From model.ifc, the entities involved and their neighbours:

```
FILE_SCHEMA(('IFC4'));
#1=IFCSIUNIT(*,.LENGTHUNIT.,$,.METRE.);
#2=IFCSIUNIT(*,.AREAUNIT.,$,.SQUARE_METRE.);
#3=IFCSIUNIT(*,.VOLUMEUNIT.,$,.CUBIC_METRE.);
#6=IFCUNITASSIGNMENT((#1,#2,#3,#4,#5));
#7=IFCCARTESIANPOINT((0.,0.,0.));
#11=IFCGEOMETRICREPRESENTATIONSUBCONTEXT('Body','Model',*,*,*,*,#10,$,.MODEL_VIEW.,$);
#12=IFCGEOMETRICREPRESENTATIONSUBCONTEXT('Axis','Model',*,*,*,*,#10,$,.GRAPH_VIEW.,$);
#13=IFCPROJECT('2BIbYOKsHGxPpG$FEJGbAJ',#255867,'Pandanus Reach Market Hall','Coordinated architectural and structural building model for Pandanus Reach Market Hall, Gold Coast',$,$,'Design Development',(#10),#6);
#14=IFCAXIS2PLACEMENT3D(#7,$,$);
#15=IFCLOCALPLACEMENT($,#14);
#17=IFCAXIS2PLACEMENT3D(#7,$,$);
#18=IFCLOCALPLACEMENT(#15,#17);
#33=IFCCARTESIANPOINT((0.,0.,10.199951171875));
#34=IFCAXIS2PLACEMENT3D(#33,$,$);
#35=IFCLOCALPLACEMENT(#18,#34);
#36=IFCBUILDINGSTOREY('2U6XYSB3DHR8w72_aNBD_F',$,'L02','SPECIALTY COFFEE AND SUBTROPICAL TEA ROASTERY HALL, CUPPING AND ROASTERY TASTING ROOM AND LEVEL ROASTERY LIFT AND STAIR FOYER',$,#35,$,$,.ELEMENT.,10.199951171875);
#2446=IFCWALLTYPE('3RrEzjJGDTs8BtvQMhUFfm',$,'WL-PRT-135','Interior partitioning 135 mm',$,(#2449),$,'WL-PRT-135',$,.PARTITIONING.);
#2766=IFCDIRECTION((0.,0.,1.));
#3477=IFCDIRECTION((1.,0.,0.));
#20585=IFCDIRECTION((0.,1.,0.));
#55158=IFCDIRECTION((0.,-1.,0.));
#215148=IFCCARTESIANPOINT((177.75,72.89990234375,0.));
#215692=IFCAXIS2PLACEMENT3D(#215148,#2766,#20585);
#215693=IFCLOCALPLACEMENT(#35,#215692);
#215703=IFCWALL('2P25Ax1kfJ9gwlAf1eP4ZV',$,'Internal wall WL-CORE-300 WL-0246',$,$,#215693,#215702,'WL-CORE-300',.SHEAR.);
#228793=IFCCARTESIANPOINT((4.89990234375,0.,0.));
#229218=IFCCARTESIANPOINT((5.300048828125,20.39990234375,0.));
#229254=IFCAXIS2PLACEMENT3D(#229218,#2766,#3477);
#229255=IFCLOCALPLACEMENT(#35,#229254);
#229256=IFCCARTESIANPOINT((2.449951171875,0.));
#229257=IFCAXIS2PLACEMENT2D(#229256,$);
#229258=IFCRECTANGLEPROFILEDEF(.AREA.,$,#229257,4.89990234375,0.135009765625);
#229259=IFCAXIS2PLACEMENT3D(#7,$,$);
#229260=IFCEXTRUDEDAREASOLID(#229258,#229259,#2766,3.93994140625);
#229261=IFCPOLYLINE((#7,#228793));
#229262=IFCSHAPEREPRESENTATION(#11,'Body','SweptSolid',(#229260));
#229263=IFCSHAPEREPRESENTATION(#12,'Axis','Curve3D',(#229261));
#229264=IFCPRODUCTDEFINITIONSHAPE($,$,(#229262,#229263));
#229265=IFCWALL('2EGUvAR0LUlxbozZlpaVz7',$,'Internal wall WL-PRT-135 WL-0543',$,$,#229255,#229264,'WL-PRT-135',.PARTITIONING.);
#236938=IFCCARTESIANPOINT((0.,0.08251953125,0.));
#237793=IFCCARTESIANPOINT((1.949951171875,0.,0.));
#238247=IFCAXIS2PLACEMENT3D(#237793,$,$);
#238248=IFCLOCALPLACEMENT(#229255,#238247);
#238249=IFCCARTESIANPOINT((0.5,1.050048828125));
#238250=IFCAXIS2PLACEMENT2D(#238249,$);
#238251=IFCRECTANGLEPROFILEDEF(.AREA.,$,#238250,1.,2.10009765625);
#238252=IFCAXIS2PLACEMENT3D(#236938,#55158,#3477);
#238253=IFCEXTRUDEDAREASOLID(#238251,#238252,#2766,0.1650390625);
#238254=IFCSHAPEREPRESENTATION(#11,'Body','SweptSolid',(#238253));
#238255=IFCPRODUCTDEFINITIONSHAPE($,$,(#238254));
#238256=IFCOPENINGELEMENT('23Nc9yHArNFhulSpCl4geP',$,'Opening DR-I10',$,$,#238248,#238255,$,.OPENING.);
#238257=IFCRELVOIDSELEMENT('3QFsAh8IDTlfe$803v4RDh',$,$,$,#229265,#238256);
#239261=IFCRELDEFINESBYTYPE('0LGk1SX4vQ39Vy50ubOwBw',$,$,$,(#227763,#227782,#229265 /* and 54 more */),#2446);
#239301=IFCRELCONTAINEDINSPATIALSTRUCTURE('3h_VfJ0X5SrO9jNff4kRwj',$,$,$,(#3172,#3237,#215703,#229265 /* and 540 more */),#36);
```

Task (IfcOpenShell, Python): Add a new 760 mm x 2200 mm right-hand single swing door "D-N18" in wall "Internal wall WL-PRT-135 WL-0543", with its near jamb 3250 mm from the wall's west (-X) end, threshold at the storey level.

```python
import numpy as np
import ifcopenshell
import ifcopenshell.api.feature
import ifcopenshell.api.geometry
import ifcopenshell.api.root
import ifcopenshell.api.spatial
import ifcopenshell.geom
import ifcopenshell.util.element
import ifcopenshell.util.placement
import ifcopenshell.util.representation
import ifcopenshell.util.shape
import ifcopenshell.util.unit

model = ifcopenshell.open("model.ifc")
unit_scale = ifcopenshell.util.unit.calculate_unit_scale(model)
settings = ifcopenshell.geom.settings()


def volume(element):
    """Net volume in cubic metres, openings subtracted."""
    shape = ifcopenshell.geom.create_shape(settings, element)
    return ifcopenshell.util.shape.get_volume(shape.geometry)


wall = model.by_guid("2EGUvAR0LUlxbozZlpaVz7")
storey = ifcopenshell.util.element.get_container(wall, ifc_class="IfcBuildingStorey")
context = ifcopenshell.util.representation.get_context(model, "Model", "Body", "MODEL_VIEW")
before = volume(wall)

width, height, from_end, sill = 0.76, 2.2, 3.25, 0.0  # metres

# The wall runs along its own X axis, and the end named is its -X end.
wall_shape = ifcopenshell.geom.create_shape(settings, wall)
x, y, z = ifcopenshell.util.shape.get_vertices(wall_shape.geometry).T
start = x.min() + from_end
face, thickness = float(y.min()), float(y.max() - y.min())
wall_matrix = ifcopenshell.util.placement.get_local_placement(wall.ObjectPlacement)
level = ifcopenshell.util.placement.get_local_placement(storey.ObjectPlacement)[2, 3]


def in_wall(x, y):
    """Placement at x, y metres in the wall's axes, at sill height."""
    matrix = wall_matrix.copy()
    matrix[:, 3] = wall_matrix @ np.array([x / unit_scale, y / unit_scale, 0.0, 1.0])
    matrix[2, 3] = level + sill / unit_scale
    return matrix


# Opening: a box that overshoots both wall faces by 50 mm.
opening = ifcopenshell.api.root.create_entity(model, ifc_class="IfcOpeningElement", predefined_type="OPENING")
box = ifcopenshell.api.geometry.add_wall_representation(
    model, context=context, length=width, height=height, thickness=thickness + 0.1
)
ifcopenshell.api.geometry.assign_representation(model, product=opening, representation=box)
ifcopenshell.api.geometry.edit_object_placement(model, product=opening, matrix=in_wall(start, face - 0.05), is_si=False)
ifcopenshell.api.feature.add_feature(model, feature=opening, element=wall)

door = ifcopenshell.api.root.create_entity(model, ifc_class="IfcDoor", name="D-N18", predefined_type="DOOR")
door.OverallWidth, door.OverallHeight = width / unit_scale, height / unit_scale
door.OperationType = "SINGLE_SWING_RIGHT"
body = ifcopenshell.api.geometry.add_door_representation(
    model,
    context=context,
    overall_width=door.OverallWidth,
    overall_height=door.OverallHeight,
    operation_type="SINGLE_SWING_RIGHT",
    lining_properties={"LiningDepth": thickness / unit_scale, "ThresholdDepth": thickness / unit_scale},
)
ifcopenshell.api.geometry.assign_representation(model, product=door, representation=body)
ifcopenshell.api.spatial.assign_container(model, products=[door], relating_structure=storey)
ifcopenshell.api.feature.add_filling(model, opening=opening, element=door)

# The lining spans the wall, so the door starts at the wall face.
ifcopenshell.api.geometry.edit_object_placement(model, product=door, matrix=in_wall(start, face), is_si=False)

after = volume(wall)

print(f"wall volume {before:.3f} -> {after:.3f} m3")

model.write("model_edited.ifc")
```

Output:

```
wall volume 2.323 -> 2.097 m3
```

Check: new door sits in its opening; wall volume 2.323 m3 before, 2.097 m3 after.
